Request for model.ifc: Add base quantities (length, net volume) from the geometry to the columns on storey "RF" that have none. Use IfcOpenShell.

First a look at what the model holds.

```python
import ifcopenshell
import ifcopenshell.util.element
import ifcopenshell.util.unit

model = ifcopenshell.open("model.ifc")
print(model.schema)
for unit_type in ("LENGTHUNIT", "AREAUNIT", "VOLUMEUNIT"):
    print(unit_type, ifcopenshell.util.unit.calculate_unit_scale(model, unit_type))
storey = next(s for s in model.by_type("IfcBuildingStorey") if s.Name == "RF")
columns = [e for e in ifcopenshell.util.element.get_decomposition(storey) if e.is_a("IfcColumn")]
for e in sorted(columns, key=lambda e: e.id()):
    print(e.id(), e.is_a(), e.Name, list(ifcopenshell.util.element.get_psets(e, qtos_only=True)), sep=" | ")
```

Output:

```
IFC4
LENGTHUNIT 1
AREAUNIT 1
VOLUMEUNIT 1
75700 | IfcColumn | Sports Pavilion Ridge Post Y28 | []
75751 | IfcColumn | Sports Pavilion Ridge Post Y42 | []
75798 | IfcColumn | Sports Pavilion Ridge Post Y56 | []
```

```python
import ifcopenshell
import ifcopenshell.api.pset
import ifcopenshell.geom
import ifcopenshell.util.element
import ifcopenshell.util.shape
import ifcopenshell.util.unit

model = ifcopenshell.open("model.ifc")
unit_scale = ifcopenshell.util.unit.calculate_unit_scale(model)
volume_scale = ifcopenshell.util.unit.calculate_unit_scale(model, "VOLUMEUNIT")
settings = ifcopenshell.geom.settings()

storey = next(s for s in model.by_type("IfcBuildingStorey") if s.Name == "RF")
columns = [e for e in ifcopenshell.util.element.get_decomposition(storey) if e.is_a("IfcColumn")]

for e in sorted(columns, key=lambda e: e.id()):
    if ifcopenshell.util.element.get_psets(e, qtos_only=True, should_inherit=False):
        continue
    # Geometry comes back in metres, in the element's own axes.
    shape = ifcopenshell.geom.create_shape(settings, e)
    values = {
        "Length": ifcopenshell.util.shape.get_z(shape.geometry) / unit_scale,
        "NetVolume": ifcopenshell.util.shape.get_volume(shape.geometry) / volume_scale,
    }
    qto = ifcopenshell.api.pset.add_qto(model, product=e, name="Qto_ColumnBaseQuantities")
    ifcopenshell.api.pset.edit_qto(model, qto=qto, properties=values)
    print(e.id(), {k: round(v, 3) for k, v in values.items()})

model.write("model_updated.ifc")
```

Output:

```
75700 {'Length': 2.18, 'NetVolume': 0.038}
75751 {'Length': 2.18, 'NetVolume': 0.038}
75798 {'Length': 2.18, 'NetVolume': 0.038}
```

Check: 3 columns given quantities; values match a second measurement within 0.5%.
